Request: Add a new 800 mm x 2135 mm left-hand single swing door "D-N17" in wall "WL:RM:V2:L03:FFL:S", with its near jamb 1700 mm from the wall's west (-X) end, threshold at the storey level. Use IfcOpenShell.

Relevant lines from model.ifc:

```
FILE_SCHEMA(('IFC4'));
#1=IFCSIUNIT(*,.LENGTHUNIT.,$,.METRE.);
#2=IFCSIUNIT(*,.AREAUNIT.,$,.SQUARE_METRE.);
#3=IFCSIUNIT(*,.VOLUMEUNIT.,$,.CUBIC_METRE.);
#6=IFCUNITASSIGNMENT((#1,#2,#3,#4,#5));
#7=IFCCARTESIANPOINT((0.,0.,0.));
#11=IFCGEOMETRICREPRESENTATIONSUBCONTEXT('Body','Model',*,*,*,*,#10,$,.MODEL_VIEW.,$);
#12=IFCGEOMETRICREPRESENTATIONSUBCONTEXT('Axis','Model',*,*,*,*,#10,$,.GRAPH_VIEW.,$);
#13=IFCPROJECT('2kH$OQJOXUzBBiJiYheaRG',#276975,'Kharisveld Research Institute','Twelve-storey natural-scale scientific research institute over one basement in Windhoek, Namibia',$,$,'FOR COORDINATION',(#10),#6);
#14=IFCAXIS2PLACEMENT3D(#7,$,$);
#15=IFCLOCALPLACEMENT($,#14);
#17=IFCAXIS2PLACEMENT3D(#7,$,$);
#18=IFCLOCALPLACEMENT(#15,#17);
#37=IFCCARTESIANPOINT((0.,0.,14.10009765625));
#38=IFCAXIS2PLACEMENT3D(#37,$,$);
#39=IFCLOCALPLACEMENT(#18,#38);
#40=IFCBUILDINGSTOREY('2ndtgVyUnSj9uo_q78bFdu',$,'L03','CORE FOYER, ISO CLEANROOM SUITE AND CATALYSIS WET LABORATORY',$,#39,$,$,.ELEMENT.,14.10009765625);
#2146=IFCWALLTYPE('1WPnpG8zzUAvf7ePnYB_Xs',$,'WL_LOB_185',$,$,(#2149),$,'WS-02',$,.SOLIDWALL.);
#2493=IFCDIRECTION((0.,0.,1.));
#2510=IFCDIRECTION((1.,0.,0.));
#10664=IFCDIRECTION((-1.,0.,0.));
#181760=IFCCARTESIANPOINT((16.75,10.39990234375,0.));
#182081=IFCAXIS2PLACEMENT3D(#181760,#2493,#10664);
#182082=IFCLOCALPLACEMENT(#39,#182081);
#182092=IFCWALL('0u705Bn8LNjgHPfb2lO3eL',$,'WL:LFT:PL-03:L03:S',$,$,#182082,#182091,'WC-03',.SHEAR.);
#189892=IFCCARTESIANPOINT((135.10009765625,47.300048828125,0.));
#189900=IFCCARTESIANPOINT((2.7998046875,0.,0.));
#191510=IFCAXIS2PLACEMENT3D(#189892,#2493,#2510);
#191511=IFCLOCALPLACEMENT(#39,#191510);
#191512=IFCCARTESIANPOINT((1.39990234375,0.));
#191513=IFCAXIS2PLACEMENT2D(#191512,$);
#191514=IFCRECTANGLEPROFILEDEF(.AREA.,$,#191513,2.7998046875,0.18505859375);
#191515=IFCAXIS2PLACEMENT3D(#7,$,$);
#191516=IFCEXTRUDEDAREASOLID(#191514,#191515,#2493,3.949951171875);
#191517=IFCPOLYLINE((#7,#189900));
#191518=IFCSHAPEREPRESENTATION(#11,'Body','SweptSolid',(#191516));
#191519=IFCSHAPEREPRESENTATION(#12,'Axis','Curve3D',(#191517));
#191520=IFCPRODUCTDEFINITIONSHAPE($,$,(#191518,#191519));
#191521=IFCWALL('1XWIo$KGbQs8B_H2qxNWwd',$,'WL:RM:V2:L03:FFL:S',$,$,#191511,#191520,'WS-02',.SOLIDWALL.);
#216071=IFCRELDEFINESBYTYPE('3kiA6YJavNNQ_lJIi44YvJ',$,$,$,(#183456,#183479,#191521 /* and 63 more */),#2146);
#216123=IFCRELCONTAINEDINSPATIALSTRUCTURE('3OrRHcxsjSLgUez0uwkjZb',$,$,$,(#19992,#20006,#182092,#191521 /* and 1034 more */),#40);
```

```python
import numpy as np
import ifcopenshell
import ifcopenshell.api.feature
import ifcopenshell.api.geometry
import ifcopenshell.api.root
import ifcopenshell.api.spatial
import ifcopenshell.geom
import ifcopenshell.util.element
import ifcopenshell.util.placement
import ifcopenshell.util.representation
import ifcopenshell.util.shape
import ifcopenshell.util.unit

model = ifcopenshell.open("model.ifc")
unit_scale = ifcopenshell.util.unit.calculate_unit_scale(model)
settings = ifcopenshell.geom.settings()


def volume(element):
    """Net volume in cubic metres, openings subtracted."""
    shape = ifcopenshell.geom.create_shape(settings, element)
    return ifcopenshell.util.shape.get_volume(shape.geometry)


wall = model.by_id(191521)
storey = ifcopenshell.util.element.get_container(wall, ifc_class="IfcBuildingStorey")
context = ifcopenshell.util.representation.get_context(model, "Model", "Body", "MODEL_VIEW")
before = volume(wall)

width, height, from_end, sill = 0.8, 2.135, 1.7, 0.0  # metres

# The wall runs along its own X axis, and the end named is its -X end.
wall_shape = ifcopenshell.geom.create_shape(settings, wall)
x, y, z = ifcopenshell.util.shape.get_vertices(wall_shape.geometry).T
start = x.min() + from_end
face, thickness = float(y.min()), float(y.max() - y.min())
wall_matrix = ifcopenshell.util.placement.get_local_placement(wall.ObjectPlacement)
level = ifcopenshell.util.placement.get_local_placement(storey.ObjectPlacement)[2, 3]


def in_wall(x, y):
    """Placement at x, y metres in the wall's axes, at sill height."""
    matrix = wall_matrix.copy()
    matrix[:, 3] = wall_matrix @ np.array([x / unit_scale, y / unit_scale, 0.0, 1.0])
    matrix[2, 3] = level + sill / unit_scale
    return matrix


# Opening: a box that overshoots both wall faces by 50 mm.
opening = ifcopenshell.api.root.create_entity(model, ifc_class="IfcOpeningElement", predefined_type="OPENING")
box = ifcopenshell.api.geometry.add_wall_representation(
    model, context=context, length=width, height=height, thickness=thickness + 0.1
)
ifcopenshell.api.geometry.assign_representation(model, product=opening, representation=box)
ifcopenshell.api.geometry.edit_object_placement(model, product=opening, matrix=in_wall(start, face - 0.05), is_si=False)
ifcopenshell.api.feature.add_feature(model, feature=opening, element=wall)

door = ifcopenshell.api.root.create_entity(model, ifc_class="IfcDoor", name="D-N17", predefined_type="DOOR")
door.OverallWidth, door.OverallHeight = width / unit_scale, height / unit_scale
door.OperationType = "SINGLE_SWING_LEFT"
body = ifcopenshell.api.geometry.add_door_representation(
    model,
    context=context,
    overall_width=door.OverallWidth,
    overall_height=door.OverallHeight,
    operation_type="SINGLE_SWING_LEFT",
    lining_properties={"LiningDepth": thickness / unit_scale, "ThresholdDepth": thickness / unit_scale},
)
ifcopenshell.api.geometry.assign_representation(model, product=door, representation=body)
ifcopenshell.api.spatial.assign_container(model, products=[door], relating_structure=storey)
ifcopenshell.api.feature.add_filling(model, opening=opening, element=door)

# The lining spans the wall, so the door starts at the wall face.
ifcopenshell.api.geometry.edit_object_placement(model, product=door, matrix=in_wall(start, face), is_si=False)

after = volume(wall)

print(f"wall volume {before:.3f} -> {after:.3f} m3")

model.write("model_rev.ifc")
```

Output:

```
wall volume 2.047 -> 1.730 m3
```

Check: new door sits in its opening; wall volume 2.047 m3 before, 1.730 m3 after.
